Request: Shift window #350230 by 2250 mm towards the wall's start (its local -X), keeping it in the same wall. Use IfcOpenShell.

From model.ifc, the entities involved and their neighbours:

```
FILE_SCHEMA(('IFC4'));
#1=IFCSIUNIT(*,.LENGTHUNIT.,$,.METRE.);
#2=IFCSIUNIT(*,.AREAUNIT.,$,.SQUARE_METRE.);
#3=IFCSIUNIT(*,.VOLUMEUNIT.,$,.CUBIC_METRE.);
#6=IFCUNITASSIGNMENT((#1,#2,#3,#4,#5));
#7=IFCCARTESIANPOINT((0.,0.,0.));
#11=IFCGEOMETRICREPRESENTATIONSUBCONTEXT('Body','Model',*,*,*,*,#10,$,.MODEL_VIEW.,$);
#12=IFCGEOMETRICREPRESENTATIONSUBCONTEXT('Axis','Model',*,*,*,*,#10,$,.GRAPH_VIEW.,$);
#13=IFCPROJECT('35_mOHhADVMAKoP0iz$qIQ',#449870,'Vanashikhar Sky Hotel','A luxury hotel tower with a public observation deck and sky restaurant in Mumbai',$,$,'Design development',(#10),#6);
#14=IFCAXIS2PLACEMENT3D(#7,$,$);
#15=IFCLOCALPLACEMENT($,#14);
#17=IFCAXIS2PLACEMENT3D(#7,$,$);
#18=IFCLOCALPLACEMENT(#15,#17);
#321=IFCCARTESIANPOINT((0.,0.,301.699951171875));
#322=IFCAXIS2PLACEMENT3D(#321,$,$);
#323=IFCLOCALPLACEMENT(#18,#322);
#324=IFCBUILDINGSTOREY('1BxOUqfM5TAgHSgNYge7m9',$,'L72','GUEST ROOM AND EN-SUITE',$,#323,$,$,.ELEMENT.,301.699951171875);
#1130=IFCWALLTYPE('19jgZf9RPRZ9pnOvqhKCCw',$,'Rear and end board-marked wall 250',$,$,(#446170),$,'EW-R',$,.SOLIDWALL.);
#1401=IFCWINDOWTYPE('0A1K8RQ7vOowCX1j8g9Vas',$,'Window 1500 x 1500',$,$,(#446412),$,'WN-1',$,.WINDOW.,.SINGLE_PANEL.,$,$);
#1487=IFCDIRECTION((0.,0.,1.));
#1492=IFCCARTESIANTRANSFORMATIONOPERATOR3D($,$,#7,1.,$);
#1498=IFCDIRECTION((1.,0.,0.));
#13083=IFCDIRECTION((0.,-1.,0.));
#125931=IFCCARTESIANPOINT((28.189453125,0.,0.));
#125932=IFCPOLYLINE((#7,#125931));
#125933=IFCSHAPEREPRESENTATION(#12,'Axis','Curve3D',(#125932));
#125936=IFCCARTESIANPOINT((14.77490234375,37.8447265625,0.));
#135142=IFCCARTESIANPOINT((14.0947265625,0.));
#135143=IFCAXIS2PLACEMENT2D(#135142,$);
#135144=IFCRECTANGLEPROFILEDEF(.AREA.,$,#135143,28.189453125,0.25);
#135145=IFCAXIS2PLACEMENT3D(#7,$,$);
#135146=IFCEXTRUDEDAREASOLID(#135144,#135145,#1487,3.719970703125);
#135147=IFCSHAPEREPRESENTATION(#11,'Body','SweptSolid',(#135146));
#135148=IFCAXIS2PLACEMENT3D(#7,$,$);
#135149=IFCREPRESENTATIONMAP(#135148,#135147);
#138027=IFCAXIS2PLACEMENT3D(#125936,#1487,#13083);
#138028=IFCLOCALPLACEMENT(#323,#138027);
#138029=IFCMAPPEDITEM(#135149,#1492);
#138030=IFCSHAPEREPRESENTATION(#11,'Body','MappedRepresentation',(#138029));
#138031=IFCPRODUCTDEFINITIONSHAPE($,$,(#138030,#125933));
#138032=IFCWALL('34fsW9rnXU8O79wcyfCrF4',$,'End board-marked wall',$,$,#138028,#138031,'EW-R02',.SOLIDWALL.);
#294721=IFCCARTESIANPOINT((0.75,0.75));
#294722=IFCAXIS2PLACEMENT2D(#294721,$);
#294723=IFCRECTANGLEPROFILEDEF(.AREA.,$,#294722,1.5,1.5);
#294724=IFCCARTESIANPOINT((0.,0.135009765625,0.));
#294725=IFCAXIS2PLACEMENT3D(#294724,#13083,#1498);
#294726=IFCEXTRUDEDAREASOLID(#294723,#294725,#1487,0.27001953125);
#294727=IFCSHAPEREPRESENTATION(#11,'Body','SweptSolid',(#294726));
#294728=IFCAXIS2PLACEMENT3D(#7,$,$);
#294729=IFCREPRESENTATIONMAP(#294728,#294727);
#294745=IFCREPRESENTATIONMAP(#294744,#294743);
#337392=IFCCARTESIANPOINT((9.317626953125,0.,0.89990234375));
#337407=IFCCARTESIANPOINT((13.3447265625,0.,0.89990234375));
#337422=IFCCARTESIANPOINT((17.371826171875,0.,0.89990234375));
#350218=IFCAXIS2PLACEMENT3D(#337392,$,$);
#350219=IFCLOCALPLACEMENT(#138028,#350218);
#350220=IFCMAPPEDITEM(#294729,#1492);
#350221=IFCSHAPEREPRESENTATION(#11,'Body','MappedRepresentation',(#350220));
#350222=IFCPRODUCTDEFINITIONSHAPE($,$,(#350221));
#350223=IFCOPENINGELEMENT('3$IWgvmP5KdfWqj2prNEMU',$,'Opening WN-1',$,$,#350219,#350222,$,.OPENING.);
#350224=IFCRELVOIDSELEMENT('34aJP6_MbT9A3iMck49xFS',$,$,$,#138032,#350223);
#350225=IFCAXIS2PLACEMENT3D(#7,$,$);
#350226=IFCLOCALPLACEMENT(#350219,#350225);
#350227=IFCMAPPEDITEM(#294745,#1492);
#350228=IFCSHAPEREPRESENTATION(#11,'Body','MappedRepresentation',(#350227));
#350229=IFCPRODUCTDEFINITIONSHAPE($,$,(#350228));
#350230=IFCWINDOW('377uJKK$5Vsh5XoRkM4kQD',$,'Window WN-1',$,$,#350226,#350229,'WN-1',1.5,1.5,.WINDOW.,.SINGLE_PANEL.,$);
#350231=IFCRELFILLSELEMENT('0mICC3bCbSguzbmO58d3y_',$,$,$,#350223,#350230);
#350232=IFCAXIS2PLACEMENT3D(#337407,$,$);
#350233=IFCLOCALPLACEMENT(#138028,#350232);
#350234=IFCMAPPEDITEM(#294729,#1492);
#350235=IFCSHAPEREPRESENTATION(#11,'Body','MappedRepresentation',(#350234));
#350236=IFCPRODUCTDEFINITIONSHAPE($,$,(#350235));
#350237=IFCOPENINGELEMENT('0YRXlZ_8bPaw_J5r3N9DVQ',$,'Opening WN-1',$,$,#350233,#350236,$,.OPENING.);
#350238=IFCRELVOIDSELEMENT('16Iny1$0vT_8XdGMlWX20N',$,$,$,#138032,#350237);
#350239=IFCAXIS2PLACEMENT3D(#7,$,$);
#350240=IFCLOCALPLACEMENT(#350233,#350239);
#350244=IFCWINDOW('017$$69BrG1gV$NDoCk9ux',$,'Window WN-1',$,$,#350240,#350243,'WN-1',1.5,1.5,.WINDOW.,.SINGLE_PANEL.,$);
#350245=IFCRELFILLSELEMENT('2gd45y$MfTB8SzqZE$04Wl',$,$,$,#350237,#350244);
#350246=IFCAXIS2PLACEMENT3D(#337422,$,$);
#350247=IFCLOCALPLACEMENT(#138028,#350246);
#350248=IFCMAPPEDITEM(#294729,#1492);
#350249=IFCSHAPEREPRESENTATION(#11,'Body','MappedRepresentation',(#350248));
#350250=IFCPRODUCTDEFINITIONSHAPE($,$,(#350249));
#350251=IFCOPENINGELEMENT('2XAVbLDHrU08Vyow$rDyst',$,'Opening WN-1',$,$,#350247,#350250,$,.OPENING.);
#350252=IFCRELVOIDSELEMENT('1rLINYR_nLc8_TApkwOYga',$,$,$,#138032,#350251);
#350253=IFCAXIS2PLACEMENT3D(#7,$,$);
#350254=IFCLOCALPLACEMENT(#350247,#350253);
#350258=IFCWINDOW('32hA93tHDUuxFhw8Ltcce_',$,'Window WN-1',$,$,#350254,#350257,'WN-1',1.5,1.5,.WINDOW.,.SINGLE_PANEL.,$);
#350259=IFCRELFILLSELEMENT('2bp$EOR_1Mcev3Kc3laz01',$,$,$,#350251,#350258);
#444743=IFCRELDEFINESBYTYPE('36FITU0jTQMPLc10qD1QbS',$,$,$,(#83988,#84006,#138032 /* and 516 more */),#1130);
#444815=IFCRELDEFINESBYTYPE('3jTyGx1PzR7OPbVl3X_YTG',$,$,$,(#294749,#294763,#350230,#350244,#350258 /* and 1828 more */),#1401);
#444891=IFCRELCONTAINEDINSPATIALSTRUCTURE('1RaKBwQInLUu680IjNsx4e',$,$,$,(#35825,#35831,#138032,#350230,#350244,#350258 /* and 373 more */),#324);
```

```python
import ifcopenshell
import ifcopenshell.api.geometry
import ifcopenshell.util.placement
import ifcopenshell.util.unit

model = ifcopenshell.open("model.ifc")
unit_scale = ifcopenshell.util.unit.calculate_unit_scale(model)

window = model.by_guid("377uJKK$5Vsh5XoRkM4kQD")
opening = window.FillsVoids[0].RelatingOpeningElement
wall = opening.VoidsElements[0].RelatingBuildingElement

wall_matrix = ifcopenshell.util.placement.get_local_placement(wall.ObjectPlacement)
shift = wall_matrix[:3, 0] * -2.25 / unit_scale
before = ifcopenshell.util.placement.get_local_placement(window.ObjectPlacement)[:3, 3].copy()

# The window is placed relative to its opening, so it follows when the opening moves.
matrix = ifcopenshell.util.placement.get_local_placement(opening.ObjectPlacement)
matrix[:3, 3] += shift
ifcopenshell.api.geometry.edit_object_placement(
    model, product=opening, matrix=matrix, is_si=False, should_transform_children=True
)

after = ifcopenshell.util.placement.get_local_placement(window.ObjectPlacement)[:3, 3]
print("window moved by", (after - before).round(3) + 0.0)

model.write("model_v2.ifc")
```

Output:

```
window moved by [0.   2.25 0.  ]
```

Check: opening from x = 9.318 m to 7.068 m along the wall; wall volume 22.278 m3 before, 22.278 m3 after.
